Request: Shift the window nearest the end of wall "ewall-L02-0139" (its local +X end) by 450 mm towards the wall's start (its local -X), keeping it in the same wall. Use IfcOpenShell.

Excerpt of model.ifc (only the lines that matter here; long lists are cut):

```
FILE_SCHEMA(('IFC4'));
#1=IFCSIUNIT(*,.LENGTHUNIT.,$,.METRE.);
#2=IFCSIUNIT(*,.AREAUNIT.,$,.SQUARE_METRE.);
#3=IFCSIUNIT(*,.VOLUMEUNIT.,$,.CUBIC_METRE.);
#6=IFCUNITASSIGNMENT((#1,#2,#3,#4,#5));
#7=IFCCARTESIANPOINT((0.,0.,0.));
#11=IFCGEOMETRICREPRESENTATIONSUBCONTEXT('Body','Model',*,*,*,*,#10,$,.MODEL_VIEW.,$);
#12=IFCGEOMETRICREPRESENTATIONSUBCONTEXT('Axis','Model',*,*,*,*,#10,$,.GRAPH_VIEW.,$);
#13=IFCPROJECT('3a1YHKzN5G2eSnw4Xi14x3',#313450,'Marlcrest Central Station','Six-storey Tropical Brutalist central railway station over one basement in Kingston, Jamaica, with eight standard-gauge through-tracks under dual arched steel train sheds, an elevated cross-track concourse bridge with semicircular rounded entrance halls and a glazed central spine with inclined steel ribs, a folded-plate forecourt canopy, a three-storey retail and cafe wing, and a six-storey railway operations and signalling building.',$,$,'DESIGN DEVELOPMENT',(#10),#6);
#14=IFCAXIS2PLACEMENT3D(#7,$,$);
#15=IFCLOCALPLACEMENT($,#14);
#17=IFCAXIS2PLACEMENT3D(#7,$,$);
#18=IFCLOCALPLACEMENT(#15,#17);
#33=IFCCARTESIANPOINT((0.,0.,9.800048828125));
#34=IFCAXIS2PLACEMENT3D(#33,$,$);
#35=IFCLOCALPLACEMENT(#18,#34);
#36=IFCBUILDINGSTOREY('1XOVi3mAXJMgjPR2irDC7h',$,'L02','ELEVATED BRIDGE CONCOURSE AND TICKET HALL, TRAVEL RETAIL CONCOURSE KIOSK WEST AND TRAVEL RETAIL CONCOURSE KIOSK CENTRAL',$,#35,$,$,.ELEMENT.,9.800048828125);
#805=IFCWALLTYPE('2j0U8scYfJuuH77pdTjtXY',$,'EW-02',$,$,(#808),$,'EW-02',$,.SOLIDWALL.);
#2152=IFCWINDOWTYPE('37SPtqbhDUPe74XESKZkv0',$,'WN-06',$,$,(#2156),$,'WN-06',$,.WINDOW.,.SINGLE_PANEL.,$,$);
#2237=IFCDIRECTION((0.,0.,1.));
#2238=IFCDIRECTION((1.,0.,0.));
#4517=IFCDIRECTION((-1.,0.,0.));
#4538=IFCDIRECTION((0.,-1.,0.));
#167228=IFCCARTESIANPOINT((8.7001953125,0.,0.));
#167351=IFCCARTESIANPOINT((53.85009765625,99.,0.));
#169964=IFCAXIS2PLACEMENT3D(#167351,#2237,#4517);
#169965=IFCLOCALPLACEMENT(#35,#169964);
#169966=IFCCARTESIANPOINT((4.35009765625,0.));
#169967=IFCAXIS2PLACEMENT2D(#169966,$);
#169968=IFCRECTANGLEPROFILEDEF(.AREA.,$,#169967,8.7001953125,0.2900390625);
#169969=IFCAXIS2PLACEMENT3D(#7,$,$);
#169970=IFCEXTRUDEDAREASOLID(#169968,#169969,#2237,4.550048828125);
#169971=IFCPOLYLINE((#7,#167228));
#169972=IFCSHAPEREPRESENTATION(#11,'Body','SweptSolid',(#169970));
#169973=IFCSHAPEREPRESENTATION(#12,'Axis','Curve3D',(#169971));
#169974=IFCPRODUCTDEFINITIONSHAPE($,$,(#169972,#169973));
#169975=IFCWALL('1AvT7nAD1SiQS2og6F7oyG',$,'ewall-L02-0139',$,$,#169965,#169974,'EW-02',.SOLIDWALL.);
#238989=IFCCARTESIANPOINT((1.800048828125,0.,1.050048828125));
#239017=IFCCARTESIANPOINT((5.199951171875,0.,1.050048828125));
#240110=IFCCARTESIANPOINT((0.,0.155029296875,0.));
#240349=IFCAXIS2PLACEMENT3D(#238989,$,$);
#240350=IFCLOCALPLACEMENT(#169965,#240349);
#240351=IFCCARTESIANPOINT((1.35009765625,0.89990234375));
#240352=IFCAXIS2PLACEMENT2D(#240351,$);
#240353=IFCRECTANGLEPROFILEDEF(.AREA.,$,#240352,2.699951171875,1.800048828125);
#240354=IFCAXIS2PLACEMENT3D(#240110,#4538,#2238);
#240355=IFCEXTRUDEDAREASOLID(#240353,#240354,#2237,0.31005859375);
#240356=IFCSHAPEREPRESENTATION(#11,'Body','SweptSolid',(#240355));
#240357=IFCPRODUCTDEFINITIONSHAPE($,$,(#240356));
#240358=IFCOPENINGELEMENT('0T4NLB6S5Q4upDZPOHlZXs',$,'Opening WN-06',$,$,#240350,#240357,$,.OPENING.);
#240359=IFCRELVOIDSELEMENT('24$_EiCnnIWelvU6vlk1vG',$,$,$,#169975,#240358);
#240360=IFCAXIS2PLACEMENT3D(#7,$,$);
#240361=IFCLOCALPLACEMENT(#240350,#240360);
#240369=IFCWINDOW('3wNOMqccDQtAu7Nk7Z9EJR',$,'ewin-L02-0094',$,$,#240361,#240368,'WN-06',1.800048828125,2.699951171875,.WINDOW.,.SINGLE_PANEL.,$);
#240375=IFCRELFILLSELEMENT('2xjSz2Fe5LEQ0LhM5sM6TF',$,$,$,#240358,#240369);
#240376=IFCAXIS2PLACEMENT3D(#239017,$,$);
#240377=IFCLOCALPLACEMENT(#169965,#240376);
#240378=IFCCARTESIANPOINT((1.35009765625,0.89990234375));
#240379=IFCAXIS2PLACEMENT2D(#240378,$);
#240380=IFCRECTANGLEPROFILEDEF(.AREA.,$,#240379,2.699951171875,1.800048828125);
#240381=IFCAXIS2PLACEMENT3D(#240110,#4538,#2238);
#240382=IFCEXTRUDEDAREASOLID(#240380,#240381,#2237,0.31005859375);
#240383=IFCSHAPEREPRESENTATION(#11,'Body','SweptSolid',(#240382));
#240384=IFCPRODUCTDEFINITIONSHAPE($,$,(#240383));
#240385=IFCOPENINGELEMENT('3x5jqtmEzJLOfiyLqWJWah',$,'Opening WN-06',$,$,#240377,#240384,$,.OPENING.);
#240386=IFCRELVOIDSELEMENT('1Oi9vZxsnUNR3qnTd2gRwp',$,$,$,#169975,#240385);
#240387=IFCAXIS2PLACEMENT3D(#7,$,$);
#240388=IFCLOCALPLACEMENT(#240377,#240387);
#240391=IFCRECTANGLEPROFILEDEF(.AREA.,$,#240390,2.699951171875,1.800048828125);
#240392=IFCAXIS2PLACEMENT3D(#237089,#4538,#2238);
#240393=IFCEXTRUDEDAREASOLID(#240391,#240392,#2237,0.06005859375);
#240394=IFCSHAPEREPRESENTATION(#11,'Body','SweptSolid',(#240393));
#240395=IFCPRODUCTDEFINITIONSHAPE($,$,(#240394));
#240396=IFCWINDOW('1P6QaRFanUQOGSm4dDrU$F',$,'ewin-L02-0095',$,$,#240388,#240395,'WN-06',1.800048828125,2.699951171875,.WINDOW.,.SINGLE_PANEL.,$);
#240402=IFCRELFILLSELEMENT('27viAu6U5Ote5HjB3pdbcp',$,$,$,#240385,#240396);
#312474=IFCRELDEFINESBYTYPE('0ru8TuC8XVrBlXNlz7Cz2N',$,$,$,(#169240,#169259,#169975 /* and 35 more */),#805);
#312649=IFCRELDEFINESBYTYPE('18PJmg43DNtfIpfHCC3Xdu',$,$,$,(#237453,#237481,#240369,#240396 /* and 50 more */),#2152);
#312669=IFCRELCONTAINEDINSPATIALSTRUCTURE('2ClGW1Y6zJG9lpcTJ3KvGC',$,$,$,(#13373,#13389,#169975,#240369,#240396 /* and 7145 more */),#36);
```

```python
import ifcopenshell
import ifcopenshell.api.geometry
import ifcopenshell.util.placement
import ifcopenshell.util.unit

model = ifcopenshell.open("model.ifc")
unit_scale = ifcopenshell.util.unit.calculate_unit_scale(model)

window = model.by_guid("1P6QaRFanUQOGSm4dDrU$F")
opening = window.FillsVoids[0].RelatingOpeningElement
wall = opening.VoidsElements[0].RelatingBuildingElement

wall_matrix = ifcopenshell.util.placement.get_local_placement(wall.ObjectPlacement)
shift = wall_matrix[:3, 0] * -0.45 / unit_scale
before = ifcopenshell.util.placement.get_local_placement(window.ObjectPlacement)[:3, 3].copy()

# The window is placed relative to its opening, so it follows when the opening moves.
matrix = ifcopenshell.util.placement.get_local_placement(opening.ObjectPlacement)
matrix[:3, 3] += shift
ifcopenshell.api.geometry.edit_object_placement(
    model, product=opening, matrix=matrix, is_si=False, should_transform_children=True
)

after = ifcopenshell.util.placement.get_local_placement(window.ObjectPlacement)[:3, 3]
print("window moved by", (after - before).round(3) + 0.0)

model.write("model_edited.ifc")
```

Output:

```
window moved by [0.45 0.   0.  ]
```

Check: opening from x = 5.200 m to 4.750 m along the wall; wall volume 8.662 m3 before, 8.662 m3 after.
